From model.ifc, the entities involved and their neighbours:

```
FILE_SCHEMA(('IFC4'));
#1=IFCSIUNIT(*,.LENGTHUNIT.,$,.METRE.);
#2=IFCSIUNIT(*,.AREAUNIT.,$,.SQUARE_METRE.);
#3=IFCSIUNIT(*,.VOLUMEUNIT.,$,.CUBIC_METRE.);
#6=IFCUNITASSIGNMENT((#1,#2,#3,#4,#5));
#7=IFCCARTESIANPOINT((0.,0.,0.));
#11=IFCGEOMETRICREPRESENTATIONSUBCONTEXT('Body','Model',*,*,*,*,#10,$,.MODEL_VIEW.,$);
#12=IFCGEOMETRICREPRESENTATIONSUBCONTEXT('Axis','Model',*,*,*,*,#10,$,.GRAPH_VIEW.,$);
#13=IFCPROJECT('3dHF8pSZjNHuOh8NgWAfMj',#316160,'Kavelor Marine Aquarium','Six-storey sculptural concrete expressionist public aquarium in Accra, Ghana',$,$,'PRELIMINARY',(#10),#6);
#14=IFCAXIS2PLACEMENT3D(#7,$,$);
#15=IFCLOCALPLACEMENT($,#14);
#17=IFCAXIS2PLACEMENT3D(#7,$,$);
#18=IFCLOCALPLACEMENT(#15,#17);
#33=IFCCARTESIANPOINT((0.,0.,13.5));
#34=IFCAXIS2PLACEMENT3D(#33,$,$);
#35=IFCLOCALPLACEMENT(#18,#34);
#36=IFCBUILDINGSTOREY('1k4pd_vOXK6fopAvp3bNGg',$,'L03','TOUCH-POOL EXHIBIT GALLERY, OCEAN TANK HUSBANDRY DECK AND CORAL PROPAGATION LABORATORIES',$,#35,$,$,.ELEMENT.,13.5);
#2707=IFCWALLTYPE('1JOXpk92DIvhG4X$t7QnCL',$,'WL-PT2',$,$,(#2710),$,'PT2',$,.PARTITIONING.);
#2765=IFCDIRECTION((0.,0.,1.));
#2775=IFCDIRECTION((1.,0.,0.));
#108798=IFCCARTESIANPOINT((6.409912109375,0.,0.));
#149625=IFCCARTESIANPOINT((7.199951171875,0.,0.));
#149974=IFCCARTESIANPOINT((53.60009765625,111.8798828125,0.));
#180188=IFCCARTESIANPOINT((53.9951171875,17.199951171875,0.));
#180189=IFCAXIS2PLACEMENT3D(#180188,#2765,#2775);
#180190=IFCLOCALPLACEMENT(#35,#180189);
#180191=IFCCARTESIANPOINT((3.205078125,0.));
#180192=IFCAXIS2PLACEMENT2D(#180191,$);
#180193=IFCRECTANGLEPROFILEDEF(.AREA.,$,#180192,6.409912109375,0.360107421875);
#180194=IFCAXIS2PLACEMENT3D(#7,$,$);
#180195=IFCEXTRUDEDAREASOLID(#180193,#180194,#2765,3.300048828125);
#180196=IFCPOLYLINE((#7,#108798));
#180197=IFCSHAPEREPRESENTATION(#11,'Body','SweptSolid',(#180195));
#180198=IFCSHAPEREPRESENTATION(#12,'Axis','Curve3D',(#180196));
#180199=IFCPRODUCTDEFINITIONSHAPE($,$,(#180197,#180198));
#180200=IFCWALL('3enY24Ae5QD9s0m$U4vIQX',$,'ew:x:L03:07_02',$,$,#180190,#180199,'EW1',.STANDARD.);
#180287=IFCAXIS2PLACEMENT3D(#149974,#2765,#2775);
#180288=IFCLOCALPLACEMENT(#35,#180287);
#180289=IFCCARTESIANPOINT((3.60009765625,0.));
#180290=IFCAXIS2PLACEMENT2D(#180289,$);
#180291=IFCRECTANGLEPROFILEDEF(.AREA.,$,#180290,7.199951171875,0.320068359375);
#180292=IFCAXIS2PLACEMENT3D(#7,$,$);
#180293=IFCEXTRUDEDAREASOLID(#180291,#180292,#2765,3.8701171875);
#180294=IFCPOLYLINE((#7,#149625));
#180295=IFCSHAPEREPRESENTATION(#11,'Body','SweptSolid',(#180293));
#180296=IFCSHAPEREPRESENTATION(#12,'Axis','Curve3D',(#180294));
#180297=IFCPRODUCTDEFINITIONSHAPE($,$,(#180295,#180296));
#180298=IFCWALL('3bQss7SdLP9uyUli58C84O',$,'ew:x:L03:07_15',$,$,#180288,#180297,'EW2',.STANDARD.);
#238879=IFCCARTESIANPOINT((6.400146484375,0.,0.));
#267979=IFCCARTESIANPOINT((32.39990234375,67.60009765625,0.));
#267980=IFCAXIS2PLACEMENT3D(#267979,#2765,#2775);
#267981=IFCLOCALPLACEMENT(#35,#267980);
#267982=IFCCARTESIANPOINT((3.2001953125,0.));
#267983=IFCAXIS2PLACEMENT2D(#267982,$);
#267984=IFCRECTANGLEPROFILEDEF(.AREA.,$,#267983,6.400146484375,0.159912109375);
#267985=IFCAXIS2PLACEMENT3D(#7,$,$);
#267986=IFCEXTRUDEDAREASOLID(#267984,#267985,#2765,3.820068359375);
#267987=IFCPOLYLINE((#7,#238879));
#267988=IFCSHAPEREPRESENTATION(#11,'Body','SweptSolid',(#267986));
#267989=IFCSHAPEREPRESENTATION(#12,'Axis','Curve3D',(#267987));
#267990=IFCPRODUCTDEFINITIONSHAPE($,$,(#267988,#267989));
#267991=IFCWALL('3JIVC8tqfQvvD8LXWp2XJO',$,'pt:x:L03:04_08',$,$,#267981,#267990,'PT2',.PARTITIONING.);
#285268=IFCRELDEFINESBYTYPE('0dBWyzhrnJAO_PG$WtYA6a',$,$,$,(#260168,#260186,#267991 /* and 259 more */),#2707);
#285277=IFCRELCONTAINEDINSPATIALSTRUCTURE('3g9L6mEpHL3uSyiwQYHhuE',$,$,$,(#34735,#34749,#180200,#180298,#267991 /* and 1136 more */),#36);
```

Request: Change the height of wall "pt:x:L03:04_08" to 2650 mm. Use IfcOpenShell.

```python
import ifcopenshell
import ifcopenshell.geom
import ifcopenshell.util.representation
import ifcopenshell.util.shape
import ifcopenshell.util.unit

model = ifcopenshell.open("model.ifc")
unit_scale = ifcopenshell.util.unit.calculate_unit_scale(model)
settings = ifcopenshell.geom.settings()


def volume(element):
    """Net volume in cubic metres, openings subtracted."""
    shape = ifcopenshell.geom.create_shape(settings, element)
    return ifcopenshell.util.shape.get_volume(shape.geometry)


wall = model.by_guid("3JIVC8tqfQvvD8LXWp2XJO")
before = volume(wall)

body = ifcopenshell.util.representation.get_representation(wall, "Model", "Body")
solid = body.Items[0]
old_height = solid.Depth
solid.Depth = 2.65 / unit_scale
after = volume(wall)

print(f"height {old_height:g} -> {solid.Depth:g}, volume {before:.3f} -> {after:.3f} m3")

model.write("model_v2.ifc")
```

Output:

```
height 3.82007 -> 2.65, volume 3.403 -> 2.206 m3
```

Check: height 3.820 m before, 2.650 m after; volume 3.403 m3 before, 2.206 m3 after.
